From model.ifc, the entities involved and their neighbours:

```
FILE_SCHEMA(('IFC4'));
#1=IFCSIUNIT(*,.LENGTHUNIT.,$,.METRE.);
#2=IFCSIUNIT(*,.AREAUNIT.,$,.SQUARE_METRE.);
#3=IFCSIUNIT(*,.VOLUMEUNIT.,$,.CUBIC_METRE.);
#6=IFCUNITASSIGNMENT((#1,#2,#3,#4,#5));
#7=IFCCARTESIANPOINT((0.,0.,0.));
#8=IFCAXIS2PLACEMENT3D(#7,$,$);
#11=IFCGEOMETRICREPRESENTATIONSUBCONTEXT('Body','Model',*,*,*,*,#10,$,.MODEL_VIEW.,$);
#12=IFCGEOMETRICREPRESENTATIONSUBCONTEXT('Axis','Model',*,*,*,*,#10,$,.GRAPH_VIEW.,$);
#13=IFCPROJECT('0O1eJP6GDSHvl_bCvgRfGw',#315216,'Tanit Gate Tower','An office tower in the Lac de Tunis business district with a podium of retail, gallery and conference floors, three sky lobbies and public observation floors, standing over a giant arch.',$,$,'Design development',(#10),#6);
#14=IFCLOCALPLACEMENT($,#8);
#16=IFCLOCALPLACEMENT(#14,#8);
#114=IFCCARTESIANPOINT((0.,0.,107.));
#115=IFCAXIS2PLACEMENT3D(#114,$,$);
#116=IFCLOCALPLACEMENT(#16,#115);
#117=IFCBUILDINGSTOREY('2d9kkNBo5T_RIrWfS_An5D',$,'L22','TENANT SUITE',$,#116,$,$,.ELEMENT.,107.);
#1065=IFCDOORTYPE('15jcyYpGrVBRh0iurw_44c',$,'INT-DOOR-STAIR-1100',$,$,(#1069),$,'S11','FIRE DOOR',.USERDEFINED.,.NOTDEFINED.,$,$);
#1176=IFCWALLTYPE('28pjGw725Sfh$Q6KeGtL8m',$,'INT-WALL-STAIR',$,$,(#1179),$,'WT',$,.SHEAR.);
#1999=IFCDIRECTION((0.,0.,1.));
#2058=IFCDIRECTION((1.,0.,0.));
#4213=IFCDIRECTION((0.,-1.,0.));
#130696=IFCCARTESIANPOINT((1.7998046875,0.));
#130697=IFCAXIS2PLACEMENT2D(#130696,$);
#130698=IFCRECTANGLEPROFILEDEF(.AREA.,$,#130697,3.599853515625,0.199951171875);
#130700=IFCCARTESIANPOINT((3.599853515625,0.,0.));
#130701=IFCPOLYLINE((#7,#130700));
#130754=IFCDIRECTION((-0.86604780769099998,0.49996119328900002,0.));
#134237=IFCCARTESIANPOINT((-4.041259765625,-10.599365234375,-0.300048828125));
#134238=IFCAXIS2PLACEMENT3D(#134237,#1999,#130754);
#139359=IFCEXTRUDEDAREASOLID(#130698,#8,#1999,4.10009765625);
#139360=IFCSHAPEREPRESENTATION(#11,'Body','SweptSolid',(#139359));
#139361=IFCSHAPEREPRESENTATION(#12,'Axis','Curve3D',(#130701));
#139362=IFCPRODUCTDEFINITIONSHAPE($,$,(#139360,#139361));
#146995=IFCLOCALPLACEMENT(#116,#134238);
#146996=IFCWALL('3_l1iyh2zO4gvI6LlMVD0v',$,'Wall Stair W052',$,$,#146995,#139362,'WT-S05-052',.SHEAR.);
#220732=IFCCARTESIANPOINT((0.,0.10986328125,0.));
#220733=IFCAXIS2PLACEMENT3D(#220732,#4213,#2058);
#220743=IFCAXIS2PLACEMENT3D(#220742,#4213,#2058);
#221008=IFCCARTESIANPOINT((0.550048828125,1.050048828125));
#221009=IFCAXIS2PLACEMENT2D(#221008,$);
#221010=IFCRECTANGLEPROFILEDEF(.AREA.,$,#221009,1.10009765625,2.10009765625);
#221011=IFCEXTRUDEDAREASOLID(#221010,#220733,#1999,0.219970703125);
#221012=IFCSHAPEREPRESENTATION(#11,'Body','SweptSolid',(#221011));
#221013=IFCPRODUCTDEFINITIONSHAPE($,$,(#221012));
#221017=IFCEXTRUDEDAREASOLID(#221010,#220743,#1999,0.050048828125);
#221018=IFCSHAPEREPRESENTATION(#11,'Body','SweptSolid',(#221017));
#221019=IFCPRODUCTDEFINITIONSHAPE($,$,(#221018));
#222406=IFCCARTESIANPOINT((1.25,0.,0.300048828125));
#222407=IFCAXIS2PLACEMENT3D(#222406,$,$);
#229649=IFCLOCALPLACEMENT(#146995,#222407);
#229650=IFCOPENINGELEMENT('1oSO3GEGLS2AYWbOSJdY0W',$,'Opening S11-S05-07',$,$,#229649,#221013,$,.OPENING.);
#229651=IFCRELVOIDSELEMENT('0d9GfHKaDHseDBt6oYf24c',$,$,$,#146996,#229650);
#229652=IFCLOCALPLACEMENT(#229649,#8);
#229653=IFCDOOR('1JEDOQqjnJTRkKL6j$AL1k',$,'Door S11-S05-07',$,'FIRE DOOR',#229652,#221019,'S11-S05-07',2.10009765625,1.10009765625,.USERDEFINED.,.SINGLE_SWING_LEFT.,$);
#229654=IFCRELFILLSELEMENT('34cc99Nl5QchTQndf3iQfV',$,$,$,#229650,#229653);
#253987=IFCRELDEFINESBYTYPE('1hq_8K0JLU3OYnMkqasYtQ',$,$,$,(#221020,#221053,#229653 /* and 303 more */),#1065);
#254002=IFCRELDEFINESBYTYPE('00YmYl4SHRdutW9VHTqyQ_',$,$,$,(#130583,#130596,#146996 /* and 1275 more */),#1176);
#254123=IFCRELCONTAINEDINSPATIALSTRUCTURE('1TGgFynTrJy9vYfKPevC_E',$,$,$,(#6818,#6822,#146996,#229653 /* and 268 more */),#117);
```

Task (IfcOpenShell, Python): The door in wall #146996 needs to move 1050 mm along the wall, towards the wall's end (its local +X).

```python
import ifcopenshell
import ifcopenshell.api.geometry
import ifcopenshell.util.placement

model = ifcopenshell.open("model.ifc")

door = model.by_guid("1JEDOQqjnJTRkKL6j$AL1k")
opening = door.FillsVoids[0].RelatingOpeningElement
wall = opening.VoidsElements[0].RelatingBuildingElement

wall_matrix = ifcopenshell.util.placement.get_local_placement(wall.ObjectPlacement)
shift = wall_matrix[:3, 0] * 1.05
before = ifcopenshell.util.placement.get_local_placement(door.ObjectPlacement)[:3, 3].copy()

# The door is placed relative to its opening, so it follows when the opening moves.
matrix = ifcopenshell.util.placement.get_local_placement(opening.ObjectPlacement)
matrix[:3, 3] += shift
ifcopenshell.api.geometry.edit_object_placement(
    model, product=opening, matrix=matrix, is_si=False, should_transform_children=True
)

after = ifcopenshell.util.placement.get_local_placement(door.ObjectPlacement)[:3, 3]
print("door moved by", (after - before).round(3) + 0.0)

model.write("model_v2.ifc")
```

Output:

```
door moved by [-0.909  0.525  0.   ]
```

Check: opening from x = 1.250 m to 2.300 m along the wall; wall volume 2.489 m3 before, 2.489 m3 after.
